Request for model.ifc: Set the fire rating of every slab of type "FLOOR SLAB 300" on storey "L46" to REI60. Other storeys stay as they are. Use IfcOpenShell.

First a look at what the model holds.

```python
import ifcopenshell
import ifcopenshell.util.element

model = ifcopenshell.open("model.ifc")
print(model.schema)
storey = next(s for s in model.by_type("IfcBuildingStorey") if s.Name == "L46")
slabs = [e for e in ifcopenshell.util.element.get_decomposition(storey) if e.is_a("IfcSlab")]
seen = {}
for e in slabs:
    element_type = ifcopenshell.util.element.get_type(e)
    key = (element_type.Name if element_type != e and element_type else None, ifcopenshell.util.element.get_pset(e, "Pset_SlabCommon", "FireRating"))
    seen[key] = seen.get(key, 0) + 1
for (name, value), count in sorted(seen.items(), key=str):
    print(count, "x", name, "|", value)
```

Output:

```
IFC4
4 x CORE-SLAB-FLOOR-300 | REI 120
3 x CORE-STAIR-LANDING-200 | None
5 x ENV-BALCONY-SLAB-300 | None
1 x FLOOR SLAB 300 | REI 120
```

```python
import ifcopenshell
import ifcopenshell.api.pset
import ifcopenshell.util.element

model = ifcopenshell.open("model.ifc")

storey = next(s for s in model.by_type("IfcBuildingStorey") if s.Name == "L46")
slabs = [e for e in ifcopenshell.util.element.get_decomposition(storey) if e.is_a("IfcSlab")]

count = 0
for e in slabs:
    element_type = ifcopenshell.util.element.get_type(e)
    if element_type in (None, e) or element_type.Name != "FLOOR SLAB 300":
        continue
    found = ifcopenshell.util.element.get_pset(e, "Pset_SlabCommon", should_inherit=False)
    if found:
        pset = model.by_id(found["id"])
        if len(ifcopenshell.util.element.get_elements_by_pset(pset)) > 1:
            pset = ifcopenshell.api.pset.unshare_pset(model, products=[e], pset=pset)[0]
    else:
        pset = ifcopenshell.api.pset.add_pset(model, product=e, name="Pset_SlabCommon")
    ifcopenshell.api.pset.edit_pset(model, pset=pset, properties={"FireRating": "REI60"})
    count += 1

print(count, "slabs updated")

model.write("model_updated.ifc")
```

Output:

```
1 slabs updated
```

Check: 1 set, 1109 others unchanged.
